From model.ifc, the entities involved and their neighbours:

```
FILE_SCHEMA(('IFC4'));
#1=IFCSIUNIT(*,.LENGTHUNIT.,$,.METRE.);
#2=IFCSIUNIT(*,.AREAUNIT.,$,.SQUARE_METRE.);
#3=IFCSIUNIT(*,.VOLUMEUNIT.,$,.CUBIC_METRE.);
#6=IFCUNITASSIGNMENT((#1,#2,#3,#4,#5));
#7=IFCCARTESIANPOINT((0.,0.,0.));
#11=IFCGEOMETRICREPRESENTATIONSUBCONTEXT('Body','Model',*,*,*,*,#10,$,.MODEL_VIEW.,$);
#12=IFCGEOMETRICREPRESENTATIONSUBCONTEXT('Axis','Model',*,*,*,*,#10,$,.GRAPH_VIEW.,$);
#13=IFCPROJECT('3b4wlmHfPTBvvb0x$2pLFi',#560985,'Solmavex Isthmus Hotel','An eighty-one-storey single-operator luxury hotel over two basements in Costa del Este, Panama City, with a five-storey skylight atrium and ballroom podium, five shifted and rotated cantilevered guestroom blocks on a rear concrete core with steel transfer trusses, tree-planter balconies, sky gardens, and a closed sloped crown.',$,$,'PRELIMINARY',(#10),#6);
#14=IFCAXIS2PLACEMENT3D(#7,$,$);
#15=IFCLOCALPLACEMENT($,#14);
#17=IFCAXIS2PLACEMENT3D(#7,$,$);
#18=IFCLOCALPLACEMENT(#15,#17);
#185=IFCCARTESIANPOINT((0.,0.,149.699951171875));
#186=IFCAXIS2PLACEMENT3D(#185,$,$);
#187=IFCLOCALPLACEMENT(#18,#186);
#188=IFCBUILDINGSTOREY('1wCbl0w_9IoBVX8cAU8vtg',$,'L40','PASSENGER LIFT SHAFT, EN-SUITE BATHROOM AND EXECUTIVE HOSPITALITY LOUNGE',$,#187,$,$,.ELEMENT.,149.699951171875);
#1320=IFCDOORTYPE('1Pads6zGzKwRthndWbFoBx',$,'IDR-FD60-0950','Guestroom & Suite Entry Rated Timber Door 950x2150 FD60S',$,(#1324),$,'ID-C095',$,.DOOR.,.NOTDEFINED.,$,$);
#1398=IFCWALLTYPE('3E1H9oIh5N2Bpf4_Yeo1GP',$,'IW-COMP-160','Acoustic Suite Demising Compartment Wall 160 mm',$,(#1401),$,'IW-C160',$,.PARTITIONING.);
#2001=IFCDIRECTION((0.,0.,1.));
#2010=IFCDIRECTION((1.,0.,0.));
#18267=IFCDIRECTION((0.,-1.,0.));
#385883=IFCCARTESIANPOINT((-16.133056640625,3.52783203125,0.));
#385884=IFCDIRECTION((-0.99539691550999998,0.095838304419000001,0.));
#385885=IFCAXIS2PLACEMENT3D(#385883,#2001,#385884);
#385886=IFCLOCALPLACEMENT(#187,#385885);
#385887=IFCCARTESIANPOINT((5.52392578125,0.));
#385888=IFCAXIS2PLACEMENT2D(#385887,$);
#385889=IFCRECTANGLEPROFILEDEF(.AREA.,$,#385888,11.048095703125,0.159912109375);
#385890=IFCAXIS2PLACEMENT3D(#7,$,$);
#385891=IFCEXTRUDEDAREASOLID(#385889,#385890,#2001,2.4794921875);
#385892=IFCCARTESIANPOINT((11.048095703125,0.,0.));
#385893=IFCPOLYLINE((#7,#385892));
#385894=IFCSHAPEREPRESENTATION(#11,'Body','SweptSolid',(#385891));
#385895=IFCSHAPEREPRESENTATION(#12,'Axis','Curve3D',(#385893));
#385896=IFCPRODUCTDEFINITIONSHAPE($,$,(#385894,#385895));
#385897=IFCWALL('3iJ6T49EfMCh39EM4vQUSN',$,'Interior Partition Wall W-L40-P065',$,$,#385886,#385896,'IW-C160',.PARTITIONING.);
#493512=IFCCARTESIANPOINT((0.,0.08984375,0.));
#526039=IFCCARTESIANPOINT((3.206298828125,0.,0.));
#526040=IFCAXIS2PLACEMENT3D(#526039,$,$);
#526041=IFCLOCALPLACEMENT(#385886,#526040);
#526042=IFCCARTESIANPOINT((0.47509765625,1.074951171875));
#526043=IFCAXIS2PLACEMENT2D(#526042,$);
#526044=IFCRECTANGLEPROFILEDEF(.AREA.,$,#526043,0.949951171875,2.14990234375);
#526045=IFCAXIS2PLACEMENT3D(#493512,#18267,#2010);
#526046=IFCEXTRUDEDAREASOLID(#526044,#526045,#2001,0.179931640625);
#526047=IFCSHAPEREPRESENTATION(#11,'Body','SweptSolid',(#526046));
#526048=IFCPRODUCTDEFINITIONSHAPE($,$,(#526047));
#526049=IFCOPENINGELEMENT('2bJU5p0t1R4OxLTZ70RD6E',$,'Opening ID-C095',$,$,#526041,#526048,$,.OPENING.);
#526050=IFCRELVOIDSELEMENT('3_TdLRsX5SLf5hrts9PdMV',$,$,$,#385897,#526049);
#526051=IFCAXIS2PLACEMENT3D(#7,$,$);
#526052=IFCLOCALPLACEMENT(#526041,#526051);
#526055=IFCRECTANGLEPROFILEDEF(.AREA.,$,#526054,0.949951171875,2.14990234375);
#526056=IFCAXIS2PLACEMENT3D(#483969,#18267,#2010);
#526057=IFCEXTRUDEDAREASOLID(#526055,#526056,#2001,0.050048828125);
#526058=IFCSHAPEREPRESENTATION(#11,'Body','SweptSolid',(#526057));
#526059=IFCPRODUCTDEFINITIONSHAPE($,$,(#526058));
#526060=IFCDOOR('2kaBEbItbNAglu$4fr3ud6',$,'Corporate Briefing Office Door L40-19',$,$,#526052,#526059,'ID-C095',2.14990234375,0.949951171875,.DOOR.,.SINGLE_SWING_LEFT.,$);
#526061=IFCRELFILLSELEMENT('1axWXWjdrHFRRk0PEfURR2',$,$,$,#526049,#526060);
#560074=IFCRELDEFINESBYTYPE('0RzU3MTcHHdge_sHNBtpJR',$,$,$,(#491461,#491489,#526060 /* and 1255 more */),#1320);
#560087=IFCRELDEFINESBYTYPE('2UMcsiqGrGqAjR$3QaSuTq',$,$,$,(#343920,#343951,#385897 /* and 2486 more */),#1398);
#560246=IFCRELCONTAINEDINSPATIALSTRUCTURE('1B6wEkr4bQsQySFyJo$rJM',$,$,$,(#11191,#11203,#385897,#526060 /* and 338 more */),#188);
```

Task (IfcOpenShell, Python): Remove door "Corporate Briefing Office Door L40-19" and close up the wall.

```python
import ifcopenshell
import ifcopenshell.api.feature
import ifcopenshell.api.root
import ifcopenshell.geom
import ifcopenshell.util.shape

model = ifcopenshell.open("model.ifc")
settings = ifcopenshell.geom.settings()


def volume(element):
    """Net volume in cubic metres, openings subtracted."""
    shape = ifcopenshell.geom.create_shape(settings, element)
    return ifcopenshell.util.shape.get_volume(shape.geometry)


door = model.by_guid("2kaBEbItbNAglu$4fr3ud6")
opening = door.FillsVoids[0].RelatingOpeningElement
wall = opening.VoidsElements[0].RelatingBuildingElement
before = volume(wall)

ifcopenshell.api.root.remove_product(model, product=door)
ifcopenshell.api.feature.remove_feature(model, feature=opening)

after = volume(wall)

print(f"wall volume {before:.3f} -> {after:.3f} m3")

model.write("model_rev.ifc")
```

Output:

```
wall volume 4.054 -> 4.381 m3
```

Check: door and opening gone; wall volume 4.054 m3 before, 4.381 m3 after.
